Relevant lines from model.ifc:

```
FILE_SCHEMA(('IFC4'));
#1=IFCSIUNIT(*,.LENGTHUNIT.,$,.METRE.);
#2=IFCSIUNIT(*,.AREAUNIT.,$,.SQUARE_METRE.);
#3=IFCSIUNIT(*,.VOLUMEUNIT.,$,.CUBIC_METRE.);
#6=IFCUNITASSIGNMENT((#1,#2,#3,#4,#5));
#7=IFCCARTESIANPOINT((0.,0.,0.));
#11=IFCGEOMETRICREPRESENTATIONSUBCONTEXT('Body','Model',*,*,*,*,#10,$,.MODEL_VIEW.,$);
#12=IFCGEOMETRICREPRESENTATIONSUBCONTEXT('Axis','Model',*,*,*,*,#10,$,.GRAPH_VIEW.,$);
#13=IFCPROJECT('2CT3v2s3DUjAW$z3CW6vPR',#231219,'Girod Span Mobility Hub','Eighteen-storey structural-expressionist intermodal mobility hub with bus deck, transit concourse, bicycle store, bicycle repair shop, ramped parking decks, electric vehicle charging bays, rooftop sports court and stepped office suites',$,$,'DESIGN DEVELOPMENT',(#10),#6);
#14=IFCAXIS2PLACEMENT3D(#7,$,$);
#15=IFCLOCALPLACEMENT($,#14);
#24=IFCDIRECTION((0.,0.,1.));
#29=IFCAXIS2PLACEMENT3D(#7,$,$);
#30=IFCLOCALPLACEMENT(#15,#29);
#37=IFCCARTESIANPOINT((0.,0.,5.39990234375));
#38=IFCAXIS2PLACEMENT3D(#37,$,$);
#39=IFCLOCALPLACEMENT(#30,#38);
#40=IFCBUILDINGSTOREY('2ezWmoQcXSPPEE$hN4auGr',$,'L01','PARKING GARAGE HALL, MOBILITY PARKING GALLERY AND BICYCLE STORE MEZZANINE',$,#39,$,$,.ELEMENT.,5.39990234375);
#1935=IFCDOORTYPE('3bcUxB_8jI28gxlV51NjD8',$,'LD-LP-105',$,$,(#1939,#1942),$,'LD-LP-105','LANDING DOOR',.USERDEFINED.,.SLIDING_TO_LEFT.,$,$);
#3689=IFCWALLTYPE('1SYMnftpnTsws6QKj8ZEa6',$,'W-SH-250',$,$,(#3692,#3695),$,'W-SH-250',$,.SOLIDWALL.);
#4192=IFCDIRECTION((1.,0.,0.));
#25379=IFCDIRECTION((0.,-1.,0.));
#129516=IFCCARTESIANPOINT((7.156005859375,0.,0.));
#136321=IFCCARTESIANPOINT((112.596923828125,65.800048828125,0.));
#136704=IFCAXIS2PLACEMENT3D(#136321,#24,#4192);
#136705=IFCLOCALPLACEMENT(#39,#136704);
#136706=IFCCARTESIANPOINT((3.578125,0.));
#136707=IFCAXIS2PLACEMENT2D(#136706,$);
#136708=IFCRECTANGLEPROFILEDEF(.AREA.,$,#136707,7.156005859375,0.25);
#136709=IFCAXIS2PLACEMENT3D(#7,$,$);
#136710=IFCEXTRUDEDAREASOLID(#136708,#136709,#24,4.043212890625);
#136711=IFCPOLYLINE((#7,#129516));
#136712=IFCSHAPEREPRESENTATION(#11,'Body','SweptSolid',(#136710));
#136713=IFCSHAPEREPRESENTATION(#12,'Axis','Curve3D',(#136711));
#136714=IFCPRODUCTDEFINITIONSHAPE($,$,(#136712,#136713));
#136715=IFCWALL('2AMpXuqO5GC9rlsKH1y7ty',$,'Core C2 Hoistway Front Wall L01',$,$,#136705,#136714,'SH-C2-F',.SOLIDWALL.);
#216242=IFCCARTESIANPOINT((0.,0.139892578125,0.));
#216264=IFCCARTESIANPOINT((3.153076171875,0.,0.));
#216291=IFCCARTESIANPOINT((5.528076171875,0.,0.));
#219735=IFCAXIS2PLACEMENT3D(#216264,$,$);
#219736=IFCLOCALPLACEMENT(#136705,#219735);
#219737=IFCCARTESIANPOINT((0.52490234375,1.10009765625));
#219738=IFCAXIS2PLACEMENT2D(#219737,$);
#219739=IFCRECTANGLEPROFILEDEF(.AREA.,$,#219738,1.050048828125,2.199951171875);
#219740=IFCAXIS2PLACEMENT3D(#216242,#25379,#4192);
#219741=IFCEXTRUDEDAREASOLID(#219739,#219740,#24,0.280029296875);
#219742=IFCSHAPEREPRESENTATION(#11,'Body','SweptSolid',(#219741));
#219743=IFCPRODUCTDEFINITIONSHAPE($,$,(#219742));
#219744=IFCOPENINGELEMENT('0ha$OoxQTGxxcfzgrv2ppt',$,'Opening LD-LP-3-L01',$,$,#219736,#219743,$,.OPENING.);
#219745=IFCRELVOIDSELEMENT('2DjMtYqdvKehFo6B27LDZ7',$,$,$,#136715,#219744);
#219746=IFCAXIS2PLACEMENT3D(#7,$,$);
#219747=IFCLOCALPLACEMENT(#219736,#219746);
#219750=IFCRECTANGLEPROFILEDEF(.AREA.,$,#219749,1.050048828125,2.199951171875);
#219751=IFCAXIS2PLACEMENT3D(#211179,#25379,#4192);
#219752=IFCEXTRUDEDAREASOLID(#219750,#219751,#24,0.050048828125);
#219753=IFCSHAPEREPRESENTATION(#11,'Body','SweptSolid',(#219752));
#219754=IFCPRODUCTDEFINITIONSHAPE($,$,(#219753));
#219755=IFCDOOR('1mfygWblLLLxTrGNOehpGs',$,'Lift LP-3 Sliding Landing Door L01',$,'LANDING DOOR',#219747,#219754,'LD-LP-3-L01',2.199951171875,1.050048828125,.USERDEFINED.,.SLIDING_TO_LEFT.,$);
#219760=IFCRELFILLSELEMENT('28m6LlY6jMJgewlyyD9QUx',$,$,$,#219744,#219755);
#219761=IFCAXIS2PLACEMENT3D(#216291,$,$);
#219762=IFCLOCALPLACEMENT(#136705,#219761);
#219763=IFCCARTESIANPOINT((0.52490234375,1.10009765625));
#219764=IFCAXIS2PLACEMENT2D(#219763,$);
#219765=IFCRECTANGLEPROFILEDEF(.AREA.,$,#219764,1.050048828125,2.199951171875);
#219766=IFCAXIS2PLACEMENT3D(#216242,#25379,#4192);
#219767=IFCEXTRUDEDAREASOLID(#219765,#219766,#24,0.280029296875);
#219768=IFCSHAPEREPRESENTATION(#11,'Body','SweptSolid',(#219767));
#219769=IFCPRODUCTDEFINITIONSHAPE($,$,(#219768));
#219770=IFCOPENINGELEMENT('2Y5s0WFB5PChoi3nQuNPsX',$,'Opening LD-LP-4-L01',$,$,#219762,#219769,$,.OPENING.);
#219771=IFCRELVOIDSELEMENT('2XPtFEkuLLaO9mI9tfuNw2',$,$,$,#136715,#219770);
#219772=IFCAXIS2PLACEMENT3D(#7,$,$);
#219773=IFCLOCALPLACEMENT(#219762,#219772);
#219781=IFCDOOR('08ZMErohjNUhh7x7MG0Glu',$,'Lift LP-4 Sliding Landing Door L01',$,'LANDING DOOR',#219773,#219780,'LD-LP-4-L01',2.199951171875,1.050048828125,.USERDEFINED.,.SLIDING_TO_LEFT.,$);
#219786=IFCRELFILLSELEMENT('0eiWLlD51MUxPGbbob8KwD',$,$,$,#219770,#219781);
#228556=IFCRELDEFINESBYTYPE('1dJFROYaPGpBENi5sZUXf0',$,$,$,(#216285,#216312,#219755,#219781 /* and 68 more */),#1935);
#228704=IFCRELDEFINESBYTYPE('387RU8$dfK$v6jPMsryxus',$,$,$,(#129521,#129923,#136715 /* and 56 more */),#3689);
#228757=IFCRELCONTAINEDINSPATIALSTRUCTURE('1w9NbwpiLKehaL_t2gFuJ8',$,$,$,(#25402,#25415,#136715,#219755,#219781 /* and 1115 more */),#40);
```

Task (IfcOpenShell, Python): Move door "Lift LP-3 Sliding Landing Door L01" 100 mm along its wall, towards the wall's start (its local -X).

```python
import ifcopenshell
import ifcopenshell.api.geometry
import ifcopenshell.util.placement
import ifcopenshell.util.unit

model = ifcopenshell.open("model.ifc")
unit_scale = ifcopenshell.util.unit.calculate_unit_scale(model)

door = model.by_id(219755)
opening = door.FillsVoids[0].RelatingOpeningElement
wall = opening.VoidsElements[0].RelatingBuildingElement

wall_matrix = ifcopenshell.util.placement.get_local_placement(wall.ObjectPlacement)
shift = wall_matrix[:3, 0] * -0.1 / unit_scale
before = ifcopenshell.util.placement.get_local_placement(door.ObjectPlacement)[:3, 3].copy()

# The door is placed relative to its opening, so it follows when the opening moves.
matrix = ifcopenshell.util.placement.get_local_placement(opening.ObjectPlacement)
matrix[:3, 3] += shift
ifcopenshell.api.geometry.edit_object_placement(
    model, product=opening, matrix=matrix, is_si=False, should_transform_children=True
)

after = ifcopenshell.util.placement.get_local_placement(door.ObjectPlacement)[:3, 3]
print("door moved by", (after - before).round(3) + 0.0)

model.write("model-out.ifc")
```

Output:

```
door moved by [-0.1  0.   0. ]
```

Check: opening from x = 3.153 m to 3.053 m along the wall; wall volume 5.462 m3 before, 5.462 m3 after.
